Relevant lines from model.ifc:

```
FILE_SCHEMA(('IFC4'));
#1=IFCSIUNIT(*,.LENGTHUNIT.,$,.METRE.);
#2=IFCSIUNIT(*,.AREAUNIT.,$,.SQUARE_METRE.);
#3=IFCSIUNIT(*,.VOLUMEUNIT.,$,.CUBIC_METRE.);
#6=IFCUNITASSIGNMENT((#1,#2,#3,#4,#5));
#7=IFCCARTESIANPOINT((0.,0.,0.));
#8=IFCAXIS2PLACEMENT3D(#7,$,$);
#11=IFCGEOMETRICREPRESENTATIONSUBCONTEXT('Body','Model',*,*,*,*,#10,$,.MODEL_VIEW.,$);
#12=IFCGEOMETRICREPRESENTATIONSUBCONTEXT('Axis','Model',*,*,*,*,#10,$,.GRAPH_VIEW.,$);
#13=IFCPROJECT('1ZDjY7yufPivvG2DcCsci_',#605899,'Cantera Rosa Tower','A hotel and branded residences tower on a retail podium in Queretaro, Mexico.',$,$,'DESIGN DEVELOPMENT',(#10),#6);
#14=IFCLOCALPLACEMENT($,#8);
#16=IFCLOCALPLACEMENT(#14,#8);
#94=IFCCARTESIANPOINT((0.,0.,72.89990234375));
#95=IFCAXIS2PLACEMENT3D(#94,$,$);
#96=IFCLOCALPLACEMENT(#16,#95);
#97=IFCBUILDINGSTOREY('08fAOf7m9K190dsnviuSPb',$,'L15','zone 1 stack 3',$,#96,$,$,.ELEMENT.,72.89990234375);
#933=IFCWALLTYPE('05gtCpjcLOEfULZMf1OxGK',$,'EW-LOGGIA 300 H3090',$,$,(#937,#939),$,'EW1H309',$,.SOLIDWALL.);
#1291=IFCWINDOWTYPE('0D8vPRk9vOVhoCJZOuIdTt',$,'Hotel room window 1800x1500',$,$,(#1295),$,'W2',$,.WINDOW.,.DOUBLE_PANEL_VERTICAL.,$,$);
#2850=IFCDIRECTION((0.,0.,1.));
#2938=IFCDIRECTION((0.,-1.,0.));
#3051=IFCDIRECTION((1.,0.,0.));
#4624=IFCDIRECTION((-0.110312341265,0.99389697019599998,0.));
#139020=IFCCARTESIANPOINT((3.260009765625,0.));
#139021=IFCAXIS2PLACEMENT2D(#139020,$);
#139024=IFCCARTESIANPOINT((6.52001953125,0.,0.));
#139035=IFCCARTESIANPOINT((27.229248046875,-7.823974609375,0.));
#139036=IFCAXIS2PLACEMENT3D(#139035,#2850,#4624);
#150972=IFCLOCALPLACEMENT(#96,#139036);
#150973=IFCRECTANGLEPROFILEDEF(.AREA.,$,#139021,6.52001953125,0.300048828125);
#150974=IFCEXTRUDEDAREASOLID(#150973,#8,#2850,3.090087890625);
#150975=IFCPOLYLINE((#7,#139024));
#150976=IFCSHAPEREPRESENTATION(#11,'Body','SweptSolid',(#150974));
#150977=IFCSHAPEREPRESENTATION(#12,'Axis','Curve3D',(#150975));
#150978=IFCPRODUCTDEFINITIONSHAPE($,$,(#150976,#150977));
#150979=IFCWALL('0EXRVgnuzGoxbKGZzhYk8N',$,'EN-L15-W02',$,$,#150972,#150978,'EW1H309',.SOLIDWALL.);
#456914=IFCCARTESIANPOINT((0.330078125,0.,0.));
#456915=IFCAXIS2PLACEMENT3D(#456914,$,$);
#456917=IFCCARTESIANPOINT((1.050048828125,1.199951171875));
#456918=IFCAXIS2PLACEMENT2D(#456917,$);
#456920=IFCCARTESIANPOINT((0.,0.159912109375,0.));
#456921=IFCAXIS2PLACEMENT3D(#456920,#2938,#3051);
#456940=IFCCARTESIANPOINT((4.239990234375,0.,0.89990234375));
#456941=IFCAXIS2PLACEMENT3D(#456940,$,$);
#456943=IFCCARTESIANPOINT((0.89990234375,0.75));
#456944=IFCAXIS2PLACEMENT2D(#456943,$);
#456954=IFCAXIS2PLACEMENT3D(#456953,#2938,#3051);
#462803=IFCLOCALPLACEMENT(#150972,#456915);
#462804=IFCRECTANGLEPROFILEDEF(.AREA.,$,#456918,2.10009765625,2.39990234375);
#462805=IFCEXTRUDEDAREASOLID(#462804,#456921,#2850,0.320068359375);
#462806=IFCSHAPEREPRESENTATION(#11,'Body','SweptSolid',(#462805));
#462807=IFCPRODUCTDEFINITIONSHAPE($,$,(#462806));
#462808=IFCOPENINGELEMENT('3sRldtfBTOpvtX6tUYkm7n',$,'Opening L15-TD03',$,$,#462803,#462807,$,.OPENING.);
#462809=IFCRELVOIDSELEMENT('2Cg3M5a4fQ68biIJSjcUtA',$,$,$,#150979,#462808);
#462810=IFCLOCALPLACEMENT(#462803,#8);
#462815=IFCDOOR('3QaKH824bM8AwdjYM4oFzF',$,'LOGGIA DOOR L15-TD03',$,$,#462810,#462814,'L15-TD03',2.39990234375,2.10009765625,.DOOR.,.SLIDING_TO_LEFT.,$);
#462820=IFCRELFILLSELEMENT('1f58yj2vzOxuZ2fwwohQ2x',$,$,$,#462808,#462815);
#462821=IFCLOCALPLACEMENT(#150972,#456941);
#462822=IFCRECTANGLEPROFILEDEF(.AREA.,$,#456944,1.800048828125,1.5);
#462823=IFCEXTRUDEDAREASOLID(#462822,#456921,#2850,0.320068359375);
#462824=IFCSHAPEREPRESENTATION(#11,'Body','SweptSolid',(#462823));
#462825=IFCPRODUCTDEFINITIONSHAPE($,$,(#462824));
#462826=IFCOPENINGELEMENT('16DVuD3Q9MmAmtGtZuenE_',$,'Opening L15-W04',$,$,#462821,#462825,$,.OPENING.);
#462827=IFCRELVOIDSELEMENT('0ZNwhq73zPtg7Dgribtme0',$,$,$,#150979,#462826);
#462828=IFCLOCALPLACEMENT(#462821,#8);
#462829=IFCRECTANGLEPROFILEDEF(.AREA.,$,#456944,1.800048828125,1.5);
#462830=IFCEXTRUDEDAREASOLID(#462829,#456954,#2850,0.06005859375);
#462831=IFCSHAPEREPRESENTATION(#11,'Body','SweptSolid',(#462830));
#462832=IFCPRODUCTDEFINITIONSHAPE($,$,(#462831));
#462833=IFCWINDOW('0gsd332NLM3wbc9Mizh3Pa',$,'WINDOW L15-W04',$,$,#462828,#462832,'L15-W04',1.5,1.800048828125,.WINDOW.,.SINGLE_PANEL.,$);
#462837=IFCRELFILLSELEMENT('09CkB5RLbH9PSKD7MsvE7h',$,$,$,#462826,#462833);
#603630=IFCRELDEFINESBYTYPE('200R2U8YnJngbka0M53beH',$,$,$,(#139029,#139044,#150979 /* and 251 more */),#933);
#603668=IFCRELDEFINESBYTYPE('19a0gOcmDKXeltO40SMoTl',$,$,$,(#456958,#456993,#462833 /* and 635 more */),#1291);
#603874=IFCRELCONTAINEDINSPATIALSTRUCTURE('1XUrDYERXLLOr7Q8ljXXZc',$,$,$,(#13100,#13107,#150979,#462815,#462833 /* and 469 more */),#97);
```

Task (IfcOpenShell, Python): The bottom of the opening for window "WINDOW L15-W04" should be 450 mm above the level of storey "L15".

```python
import numpy as np
import ifcopenshell
import ifcopenshell.api.geometry
import ifcopenshell.geom
import ifcopenshell.util.element
import ifcopenshell.util.placement
import ifcopenshell.util.shape
import ifcopenshell.util.unit

model = ifcopenshell.open("model.ifc")
unit_scale = ifcopenshell.util.unit.calculate_unit_scale(model)

window = model.by_guid("0gsd332NLM3wbc9Mizh3Pa")
opening = window.FillsVoids[0].RelatingOpeningElement
storey = ifcopenshell.util.element.get_container(window, ifc_class="IfcBuildingStorey")
level = ifcopenshell.util.placement.get_local_placement(storey.ObjectPlacement)[2, 3]

# The opening's origin need not be at the sill, so measure its lowest point.
shape = ifcopenshell.geom.create_shape(ifcopenshell.geom.settings(), opening)
bottom = ifcopenshell.util.shape.get_shape_bottom_elevation(shape, shape.geometry) / unit_scale
dz = level + 0.45 / unit_scale - bottom

shift = np.array([0.0, 0.0, dz])
# The window is placed relative to its opening, so it follows when the opening moves.
matrix = ifcopenshell.util.placement.get_local_placement(opening.ObjectPlacement)
matrix[:3, 3] += shift
ifcopenshell.api.geometry.edit_object_placement(
    model, product=opening, matrix=matrix, is_si=False, should_transform_children=True
)

print(f"moved by {dz * unit_scale:+.3f} m")

model.write("model_v2.ifc")
```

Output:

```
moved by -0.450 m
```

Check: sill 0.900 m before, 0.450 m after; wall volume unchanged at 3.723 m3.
